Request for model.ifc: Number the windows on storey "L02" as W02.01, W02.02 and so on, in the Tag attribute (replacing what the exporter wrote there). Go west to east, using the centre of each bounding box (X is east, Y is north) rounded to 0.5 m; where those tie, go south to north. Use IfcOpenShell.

First a look at what the model holds.

```python
import ifcopenshell
import ifcopenshell.util.element
import ifcopenshell.util.placement

model = ifcopenshell.open("model.ifc")
print(model.schema)
storey = next(s for s in model.by_type("IfcBuildingStorey") if s.Name == "L02")
windows = [e for e in ifcopenshell.util.element.get_decomposition(storey) if e.is_a("IfcWindow")]
for e in sorted(windows, key=lambda e: e.id()):
    origin = ifcopenshell.util.placement.get_local_placement(e.ObjectPlacement)[:3, 3]
    print(e.id(), e.Tag, e.Name, origin.round(2) + 0.0, sep=" | ")
```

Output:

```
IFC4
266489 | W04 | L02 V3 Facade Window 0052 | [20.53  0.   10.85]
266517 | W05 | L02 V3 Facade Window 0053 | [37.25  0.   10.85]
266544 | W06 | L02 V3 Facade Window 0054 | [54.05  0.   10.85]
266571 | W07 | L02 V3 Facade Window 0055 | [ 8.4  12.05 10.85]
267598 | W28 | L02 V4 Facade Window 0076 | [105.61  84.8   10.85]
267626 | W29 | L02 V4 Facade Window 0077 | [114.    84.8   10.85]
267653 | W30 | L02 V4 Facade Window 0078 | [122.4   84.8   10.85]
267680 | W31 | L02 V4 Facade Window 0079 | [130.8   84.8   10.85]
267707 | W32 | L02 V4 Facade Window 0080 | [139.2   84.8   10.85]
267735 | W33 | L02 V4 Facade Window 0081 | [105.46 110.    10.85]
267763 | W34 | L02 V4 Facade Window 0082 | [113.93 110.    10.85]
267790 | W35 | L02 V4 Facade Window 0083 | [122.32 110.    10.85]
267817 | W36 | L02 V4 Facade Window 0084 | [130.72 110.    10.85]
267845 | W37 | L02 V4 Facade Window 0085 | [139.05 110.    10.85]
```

```python
import ifcopenshell
import ifcopenshell.geom
import ifcopenshell.util.element
import ifcopenshell.util.shape

model = ifcopenshell.open("model.ifc")
settings = ifcopenshell.geom.settings()
settings.set("use-world-coords", True)


def centre(element):
    shape = ifcopenshell.geom.create_shape(settings, element)
    return ifcopenshell.util.shape.get_bbox_centroid(shape.geometry)


storey = next(s for s in model.by_type("IfcBuildingStorey") if s.Name == "L02")
windows = [e for e in ifcopenshell.util.element.get_decomposition(storey) if e.is_a("IfcWindow")]

# Insertion points can sit at a corner or the storey origin, so sort by the geometry (in metres).
centres = {e: centre(e) for e in windows}
windows.sort(key=lambda e: (round(centres[e][0] / 0.5), centres[e][1]))

for i, e in enumerate(windows, start=1):
    number = f"W02.{i:02d}"
    e.Tag = number
    print(e.id(), number)

model.write("model_edited.ifc")
```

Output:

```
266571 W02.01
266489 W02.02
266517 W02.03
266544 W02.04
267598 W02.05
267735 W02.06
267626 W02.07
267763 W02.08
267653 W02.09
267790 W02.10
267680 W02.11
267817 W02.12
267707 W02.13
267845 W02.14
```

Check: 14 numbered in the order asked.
